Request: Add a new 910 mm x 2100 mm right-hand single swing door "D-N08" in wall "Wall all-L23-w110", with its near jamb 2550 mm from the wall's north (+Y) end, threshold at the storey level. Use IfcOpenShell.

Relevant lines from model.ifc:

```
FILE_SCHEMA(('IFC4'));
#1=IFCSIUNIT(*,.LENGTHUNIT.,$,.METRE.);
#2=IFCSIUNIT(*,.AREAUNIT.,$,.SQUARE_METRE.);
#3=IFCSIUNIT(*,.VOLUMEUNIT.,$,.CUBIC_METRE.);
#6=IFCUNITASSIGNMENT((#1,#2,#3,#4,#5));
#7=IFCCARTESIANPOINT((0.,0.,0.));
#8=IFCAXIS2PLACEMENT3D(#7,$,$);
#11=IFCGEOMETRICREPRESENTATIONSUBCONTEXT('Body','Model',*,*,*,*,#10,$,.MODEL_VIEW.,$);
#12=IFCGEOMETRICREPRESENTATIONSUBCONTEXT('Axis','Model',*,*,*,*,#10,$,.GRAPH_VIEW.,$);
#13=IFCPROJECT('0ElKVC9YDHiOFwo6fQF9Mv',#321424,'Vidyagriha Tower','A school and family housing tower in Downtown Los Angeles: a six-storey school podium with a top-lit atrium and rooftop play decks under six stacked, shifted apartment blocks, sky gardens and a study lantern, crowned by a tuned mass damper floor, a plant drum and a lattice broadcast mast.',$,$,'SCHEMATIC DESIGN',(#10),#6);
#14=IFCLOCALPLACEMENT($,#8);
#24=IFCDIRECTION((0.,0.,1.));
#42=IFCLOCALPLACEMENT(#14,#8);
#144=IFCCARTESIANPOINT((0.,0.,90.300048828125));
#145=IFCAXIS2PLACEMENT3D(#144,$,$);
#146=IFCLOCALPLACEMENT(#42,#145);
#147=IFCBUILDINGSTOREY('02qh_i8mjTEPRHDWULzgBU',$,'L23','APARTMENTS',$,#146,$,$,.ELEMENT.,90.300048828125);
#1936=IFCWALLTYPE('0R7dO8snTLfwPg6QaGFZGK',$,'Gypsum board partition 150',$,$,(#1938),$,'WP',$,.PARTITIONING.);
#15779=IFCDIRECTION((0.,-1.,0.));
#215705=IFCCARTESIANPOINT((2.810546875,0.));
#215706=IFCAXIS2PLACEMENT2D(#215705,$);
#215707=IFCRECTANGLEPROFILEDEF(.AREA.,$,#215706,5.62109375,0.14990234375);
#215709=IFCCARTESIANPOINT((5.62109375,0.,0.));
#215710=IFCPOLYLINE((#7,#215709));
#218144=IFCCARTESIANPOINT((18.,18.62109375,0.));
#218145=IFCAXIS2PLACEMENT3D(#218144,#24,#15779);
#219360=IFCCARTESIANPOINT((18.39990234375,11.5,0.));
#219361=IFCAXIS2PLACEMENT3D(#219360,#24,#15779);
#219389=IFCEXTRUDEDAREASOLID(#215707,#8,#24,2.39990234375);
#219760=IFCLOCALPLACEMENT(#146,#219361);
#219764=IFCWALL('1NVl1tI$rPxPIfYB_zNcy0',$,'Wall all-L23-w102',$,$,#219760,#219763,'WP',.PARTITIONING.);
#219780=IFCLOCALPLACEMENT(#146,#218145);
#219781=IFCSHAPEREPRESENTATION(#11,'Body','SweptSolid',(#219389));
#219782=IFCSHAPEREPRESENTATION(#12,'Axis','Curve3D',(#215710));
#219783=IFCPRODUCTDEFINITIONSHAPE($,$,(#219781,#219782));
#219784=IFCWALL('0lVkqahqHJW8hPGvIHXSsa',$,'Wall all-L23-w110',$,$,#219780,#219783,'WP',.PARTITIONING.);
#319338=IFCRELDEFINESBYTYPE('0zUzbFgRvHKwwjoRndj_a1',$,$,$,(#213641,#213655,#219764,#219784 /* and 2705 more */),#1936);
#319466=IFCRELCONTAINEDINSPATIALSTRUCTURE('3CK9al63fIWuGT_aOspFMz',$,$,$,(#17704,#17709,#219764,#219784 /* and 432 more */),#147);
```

```python
import numpy as np
import ifcopenshell
import ifcopenshell.api.feature
import ifcopenshell.api.geometry
import ifcopenshell.api.root
import ifcopenshell.api.spatial
import ifcopenshell.geom
import ifcopenshell.util.element
import ifcopenshell.util.placement
import ifcopenshell.util.representation
import ifcopenshell.util.shape
import ifcopenshell.util.unit

model = ifcopenshell.open("model.ifc")
unit_scale = ifcopenshell.util.unit.calculate_unit_scale(model)
settings = ifcopenshell.geom.settings()


def volume(element):
    """Net volume in cubic metres, openings subtracted."""
    shape = ifcopenshell.geom.create_shape(settings, element)
    return ifcopenshell.util.shape.get_volume(shape.geometry)


wall = model.by_id(219784)
storey = ifcopenshell.util.element.get_container(wall, ifc_class="IfcBuildingStorey")
context = ifcopenshell.util.representation.get_context(model, "Model", "Body", "MODEL_VIEW")
before = volume(wall)

width, height, from_end, sill = 0.91, 2.1, 2.55, 0.0  # metres

# The wall runs along its own X axis, and the end named is its -X end.
wall_shape = ifcopenshell.geom.create_shape(settings, wall)
x, y, z = ifcopenshell.util.shape.get_vertices(wall_shape.geometry).T
start = x.min() + from_end
face, thickness = float(y.min()), float(y.max() - y.min())
wall_matrix = ifcopenshell.util.placement.get_local_placement(wall.ObjectPlacement)
level = ifcopenshell.util.placement.get_local_placement(storey.ObjectPlacement)[2, 3]


def in_wall(x, y):
    """Placement at x, y metres in the wall's axes, at sill height."""
    matrix = wall_matrix.copy()
    matrix[:, 3] = wall_matrix @ np.array([x / unit_scale, y / unit_scale, 0.0, 1.0])
    matrix[2, 3] = level + sill / unit_scale
    return matrix


# Opening: a box that overshoots both wall faces by 50 mm.
opening = ifcopenshell.api.root.create_entity(model, ifc_class="IfcOpeningElement", predefined_type="OPENING")
box = ifcopenshell.api.geometry.add_wall_representation(
    model, context=context, length=width, height=height, thickness=thickness + 0.1
)
ifcopenshell.api.geometry.assign_representation(model, product=opening, representation=box)
ifcopenshell.api.geometry.edit_object_placement(model, product=opening, matrix=in_wall(start, face - 0.05), is_si=False)
ifcopenshell.api.feature.add_feature(model, feature=opening, element=wall)

door = ifcopenshell.api.root.create_entity(model, ifc_class="IfcDoor", name="D-N08", predefined_type="DOOR")
door.OverallWidth, door.OverallHeight = width / unit_scale, height / unit_scale
door.OperationType = "SINGLE_SWING_RIGHT"
body = ifcopenshell.api.geometry.add_door_representation(
    model,
    context=context,
    overall_width=door.OverallWidth,
    overall_height=door.OverallHeight,
    operation_type="SINGLE_SWING_RIGHT",
    lining_properties={"LiningDepth": thickness / unit_scale, "ThresholdDepth": thickness / unit_scale},
)
ifcopenshell.api.geometry.assign_representation(model, product=door, representation=body)
ifcopenshell.api.spatial.assign_container(model, products=[door], relating_structure=storey)
ifcopenshell.api.feature.add_filling(model, opening=opening, element=door)

# The lining spans the wall, so the door starts at the wall face.
ifcopenshell.api.geometry.edit_object_placement(model, product=door, matrix=in_wall(start, face), is_si=False)

after = volume(wall)

print(f"wall volume {before:.3f} -> {after:.3f} m3")

model.write("model_v2.ifc")
```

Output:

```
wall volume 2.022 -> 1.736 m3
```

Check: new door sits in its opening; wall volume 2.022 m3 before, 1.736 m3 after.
